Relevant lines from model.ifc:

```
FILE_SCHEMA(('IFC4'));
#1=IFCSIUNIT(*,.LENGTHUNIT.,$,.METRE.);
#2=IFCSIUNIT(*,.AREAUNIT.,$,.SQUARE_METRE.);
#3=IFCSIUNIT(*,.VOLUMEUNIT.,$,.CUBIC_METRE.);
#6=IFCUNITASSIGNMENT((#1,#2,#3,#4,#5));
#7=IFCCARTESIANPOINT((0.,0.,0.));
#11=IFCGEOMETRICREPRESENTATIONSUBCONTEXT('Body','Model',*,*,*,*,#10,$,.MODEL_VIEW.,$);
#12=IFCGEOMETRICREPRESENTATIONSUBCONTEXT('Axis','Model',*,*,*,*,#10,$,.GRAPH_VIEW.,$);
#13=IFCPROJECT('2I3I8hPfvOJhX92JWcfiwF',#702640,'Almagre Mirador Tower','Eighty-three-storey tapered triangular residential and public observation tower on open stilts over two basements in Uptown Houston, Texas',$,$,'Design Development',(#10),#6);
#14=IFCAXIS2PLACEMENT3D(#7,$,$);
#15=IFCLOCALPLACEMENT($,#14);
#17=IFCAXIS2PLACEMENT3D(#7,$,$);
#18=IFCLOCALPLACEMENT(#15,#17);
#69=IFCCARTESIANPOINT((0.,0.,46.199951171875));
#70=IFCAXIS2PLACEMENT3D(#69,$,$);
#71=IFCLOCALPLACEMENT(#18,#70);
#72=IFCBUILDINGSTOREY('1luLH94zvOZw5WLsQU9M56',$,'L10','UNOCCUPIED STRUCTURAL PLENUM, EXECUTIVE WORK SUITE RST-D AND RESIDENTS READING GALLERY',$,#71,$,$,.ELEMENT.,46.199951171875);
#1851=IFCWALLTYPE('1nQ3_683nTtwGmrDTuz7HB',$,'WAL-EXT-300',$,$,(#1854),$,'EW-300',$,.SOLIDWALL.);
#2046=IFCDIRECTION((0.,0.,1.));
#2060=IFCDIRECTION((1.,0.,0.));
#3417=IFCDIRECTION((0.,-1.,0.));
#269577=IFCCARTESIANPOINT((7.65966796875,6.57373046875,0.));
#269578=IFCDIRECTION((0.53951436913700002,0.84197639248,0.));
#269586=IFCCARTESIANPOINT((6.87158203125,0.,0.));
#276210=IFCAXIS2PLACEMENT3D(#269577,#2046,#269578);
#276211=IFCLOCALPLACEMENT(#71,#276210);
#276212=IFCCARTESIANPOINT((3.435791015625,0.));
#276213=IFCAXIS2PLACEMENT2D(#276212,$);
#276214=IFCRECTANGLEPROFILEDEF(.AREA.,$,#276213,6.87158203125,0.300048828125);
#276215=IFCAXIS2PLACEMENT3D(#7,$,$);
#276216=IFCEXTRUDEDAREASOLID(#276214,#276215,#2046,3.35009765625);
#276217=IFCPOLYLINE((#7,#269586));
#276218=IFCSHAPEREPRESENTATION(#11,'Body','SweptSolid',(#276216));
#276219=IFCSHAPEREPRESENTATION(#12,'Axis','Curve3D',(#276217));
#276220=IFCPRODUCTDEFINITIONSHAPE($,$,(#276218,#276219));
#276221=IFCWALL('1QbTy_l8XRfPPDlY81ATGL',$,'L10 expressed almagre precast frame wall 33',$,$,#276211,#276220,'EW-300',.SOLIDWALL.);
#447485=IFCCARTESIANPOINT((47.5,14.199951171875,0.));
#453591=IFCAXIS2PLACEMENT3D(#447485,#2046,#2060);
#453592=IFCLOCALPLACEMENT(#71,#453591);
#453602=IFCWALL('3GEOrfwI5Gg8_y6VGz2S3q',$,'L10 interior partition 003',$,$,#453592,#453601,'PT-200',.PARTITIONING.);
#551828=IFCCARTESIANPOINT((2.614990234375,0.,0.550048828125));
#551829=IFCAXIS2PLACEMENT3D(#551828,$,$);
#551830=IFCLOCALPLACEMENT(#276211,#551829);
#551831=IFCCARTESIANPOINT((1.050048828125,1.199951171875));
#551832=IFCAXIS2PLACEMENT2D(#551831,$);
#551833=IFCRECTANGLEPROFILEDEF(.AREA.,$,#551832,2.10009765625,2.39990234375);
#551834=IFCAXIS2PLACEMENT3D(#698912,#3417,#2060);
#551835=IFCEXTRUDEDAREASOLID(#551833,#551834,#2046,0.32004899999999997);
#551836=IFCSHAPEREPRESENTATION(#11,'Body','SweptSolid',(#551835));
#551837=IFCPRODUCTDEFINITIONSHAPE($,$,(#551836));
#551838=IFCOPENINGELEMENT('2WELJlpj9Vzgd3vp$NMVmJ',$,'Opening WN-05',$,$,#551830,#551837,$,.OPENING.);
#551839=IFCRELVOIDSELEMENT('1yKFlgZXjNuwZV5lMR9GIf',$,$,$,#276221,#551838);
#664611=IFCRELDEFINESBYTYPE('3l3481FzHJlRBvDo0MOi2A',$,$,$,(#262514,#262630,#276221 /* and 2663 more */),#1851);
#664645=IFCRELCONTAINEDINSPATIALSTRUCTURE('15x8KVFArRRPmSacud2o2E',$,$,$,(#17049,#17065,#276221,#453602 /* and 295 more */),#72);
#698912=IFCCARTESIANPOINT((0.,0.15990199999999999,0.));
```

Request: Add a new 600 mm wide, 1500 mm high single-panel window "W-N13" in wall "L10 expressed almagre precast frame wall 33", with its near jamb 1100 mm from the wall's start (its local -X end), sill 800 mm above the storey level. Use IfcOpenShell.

```python
import numpy as np
import ifcopenshell
import ifcopenshell.api.feature
import ifcopenshell.api.geometry
import ifcopenshell.api.root
import ifcopenshell.api.spatial
import ifcopenshell.geom
import ifcopenshell.util.element
import ifcopenshell.util.placement
import ifcopenshell.util.representation
import ifcopenshell.util.shape
import ifcopenshell.util.unit

model = ifcopenshell.open("model.ifc")
unit_scale = ifcopenshell.util.unit.calculate_unit_scale(model)
settings = ifcopenshell.geom.settings()


def volume(element):
    """Net volume in cubic metres, openings subtracted."""
    shape = ifcopenshell.geom.create_shape(settings, element)
    return ifcopenshell.util.shape.get_volume(shape.geometry)


wall = model.by_id(276221)
storey = ifcopenshell.util.element.get_container(wall, ifc_class="IfcBuildingStorey")
context = ifcopenshell.util.representation.get_context(model, "Model", "Body", "MODEL_VIEW")
before = volume(wall)

width, height, from_end, sill = 0.6, 1.5, 1.1, 0.8  # metres

# The wall runs along its own X axis, and the end named is its -X end.
wall_shape = ifcopenshell.geom.create_shape(settings, wall)
x, y, z = ifcopenshell.util.shape.get_vertices(wall_shape.geometry).T
start = x.min() + from_end
face, thickness = float(y.min()), float(y.max() - y.min())
wall_matrix = ifcopenshell.util.placement.get_local_placement(wall.ObjectPlacement)
level = ifcopenshell.util.placement.get_local_placement(storey.ObjectPlacement)[2, 3]


def in_wall(x, y):
    """Placement at x, y metres in the wall's axes, at sill height."""
    matrix = wall_matrix.copy()
    matrix[:, 3] = wall_matrix @ np.array([x / unit_scale, y / unit_scale, 0.0, 1.0])
    matrix[2, 3] = level + sill / unit_scale
    return matrix


# Opening: a box that overshoots both wall faces by 50 mm.
opening = ifcopenshell.api.root.create_entity(model, ifc_class="IfcOpeningElement", predefined_type="OPENING")
box = ifcopenshell.api.geometry.add_wall_representation(
    model, context=context, length=width, height=height, thickness=thickness + 0.1
)
ifcopenshell.api.geometry.assign_representation(model, product=opening, representation=box)
ifcopenshell.api.geometry.edit_object_placement(model, product=opening, matrix=in_wall(start, face - 0.05), is_si=False)
ifcopenshell.api.feature.add_feature(model, feature=opening, element=wall)

window = ifcopenshell.api.root.create_entity(model, ifc_class="IfcWindow", name="W-N13", predefined_type="WINDOW")
window.OverallWidth, window.OverallHeight = width / unit_scale, height / unit_scale
window.PartitioningType = "SINGLE_PANEL"
body = ifcopenshell.api.geometry.add_window_representation(
    model,
    context=context,
    overall_width=window.OverallWidth,
    overall_height=window.OverallHeight,
    partition_type="SINGLE_PANEL",
)
ifcopenshell.api.geometry.assign_representation(model, product=window, representation=body)
ifcopenshell.api.spatial.assign_container(model, products=[window], relating_structure=storey)
ifcopenshell.api.feature.add_filling(model, opening=opening, element=window)

# Centre the window in the wall's thickness.
ifcopenshell.api.geometry.edit_object_placement(model, product=window, matrix=in_wall(start, face), is_si=False)
window_shape = ifcopenshell.geom.create_shape(settings, window)
depth = ifcopenshell.util.shape.get_vertices(window_shape.geometry)[:, 1]
offset = face + thickness / 2 - (depth.min() + depth.max()) / 2
ifcopenshell.api.geometry.edit_object_placement(model, product=window, matrix=in_wall(start, offset), is_si=False)

after = volume(wall)

print(f"wall volume {before:.3f} -> {after:.3f} m3")

model.write("model_updated.ifc")
```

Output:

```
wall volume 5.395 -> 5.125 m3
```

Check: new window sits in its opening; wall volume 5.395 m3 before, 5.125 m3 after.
